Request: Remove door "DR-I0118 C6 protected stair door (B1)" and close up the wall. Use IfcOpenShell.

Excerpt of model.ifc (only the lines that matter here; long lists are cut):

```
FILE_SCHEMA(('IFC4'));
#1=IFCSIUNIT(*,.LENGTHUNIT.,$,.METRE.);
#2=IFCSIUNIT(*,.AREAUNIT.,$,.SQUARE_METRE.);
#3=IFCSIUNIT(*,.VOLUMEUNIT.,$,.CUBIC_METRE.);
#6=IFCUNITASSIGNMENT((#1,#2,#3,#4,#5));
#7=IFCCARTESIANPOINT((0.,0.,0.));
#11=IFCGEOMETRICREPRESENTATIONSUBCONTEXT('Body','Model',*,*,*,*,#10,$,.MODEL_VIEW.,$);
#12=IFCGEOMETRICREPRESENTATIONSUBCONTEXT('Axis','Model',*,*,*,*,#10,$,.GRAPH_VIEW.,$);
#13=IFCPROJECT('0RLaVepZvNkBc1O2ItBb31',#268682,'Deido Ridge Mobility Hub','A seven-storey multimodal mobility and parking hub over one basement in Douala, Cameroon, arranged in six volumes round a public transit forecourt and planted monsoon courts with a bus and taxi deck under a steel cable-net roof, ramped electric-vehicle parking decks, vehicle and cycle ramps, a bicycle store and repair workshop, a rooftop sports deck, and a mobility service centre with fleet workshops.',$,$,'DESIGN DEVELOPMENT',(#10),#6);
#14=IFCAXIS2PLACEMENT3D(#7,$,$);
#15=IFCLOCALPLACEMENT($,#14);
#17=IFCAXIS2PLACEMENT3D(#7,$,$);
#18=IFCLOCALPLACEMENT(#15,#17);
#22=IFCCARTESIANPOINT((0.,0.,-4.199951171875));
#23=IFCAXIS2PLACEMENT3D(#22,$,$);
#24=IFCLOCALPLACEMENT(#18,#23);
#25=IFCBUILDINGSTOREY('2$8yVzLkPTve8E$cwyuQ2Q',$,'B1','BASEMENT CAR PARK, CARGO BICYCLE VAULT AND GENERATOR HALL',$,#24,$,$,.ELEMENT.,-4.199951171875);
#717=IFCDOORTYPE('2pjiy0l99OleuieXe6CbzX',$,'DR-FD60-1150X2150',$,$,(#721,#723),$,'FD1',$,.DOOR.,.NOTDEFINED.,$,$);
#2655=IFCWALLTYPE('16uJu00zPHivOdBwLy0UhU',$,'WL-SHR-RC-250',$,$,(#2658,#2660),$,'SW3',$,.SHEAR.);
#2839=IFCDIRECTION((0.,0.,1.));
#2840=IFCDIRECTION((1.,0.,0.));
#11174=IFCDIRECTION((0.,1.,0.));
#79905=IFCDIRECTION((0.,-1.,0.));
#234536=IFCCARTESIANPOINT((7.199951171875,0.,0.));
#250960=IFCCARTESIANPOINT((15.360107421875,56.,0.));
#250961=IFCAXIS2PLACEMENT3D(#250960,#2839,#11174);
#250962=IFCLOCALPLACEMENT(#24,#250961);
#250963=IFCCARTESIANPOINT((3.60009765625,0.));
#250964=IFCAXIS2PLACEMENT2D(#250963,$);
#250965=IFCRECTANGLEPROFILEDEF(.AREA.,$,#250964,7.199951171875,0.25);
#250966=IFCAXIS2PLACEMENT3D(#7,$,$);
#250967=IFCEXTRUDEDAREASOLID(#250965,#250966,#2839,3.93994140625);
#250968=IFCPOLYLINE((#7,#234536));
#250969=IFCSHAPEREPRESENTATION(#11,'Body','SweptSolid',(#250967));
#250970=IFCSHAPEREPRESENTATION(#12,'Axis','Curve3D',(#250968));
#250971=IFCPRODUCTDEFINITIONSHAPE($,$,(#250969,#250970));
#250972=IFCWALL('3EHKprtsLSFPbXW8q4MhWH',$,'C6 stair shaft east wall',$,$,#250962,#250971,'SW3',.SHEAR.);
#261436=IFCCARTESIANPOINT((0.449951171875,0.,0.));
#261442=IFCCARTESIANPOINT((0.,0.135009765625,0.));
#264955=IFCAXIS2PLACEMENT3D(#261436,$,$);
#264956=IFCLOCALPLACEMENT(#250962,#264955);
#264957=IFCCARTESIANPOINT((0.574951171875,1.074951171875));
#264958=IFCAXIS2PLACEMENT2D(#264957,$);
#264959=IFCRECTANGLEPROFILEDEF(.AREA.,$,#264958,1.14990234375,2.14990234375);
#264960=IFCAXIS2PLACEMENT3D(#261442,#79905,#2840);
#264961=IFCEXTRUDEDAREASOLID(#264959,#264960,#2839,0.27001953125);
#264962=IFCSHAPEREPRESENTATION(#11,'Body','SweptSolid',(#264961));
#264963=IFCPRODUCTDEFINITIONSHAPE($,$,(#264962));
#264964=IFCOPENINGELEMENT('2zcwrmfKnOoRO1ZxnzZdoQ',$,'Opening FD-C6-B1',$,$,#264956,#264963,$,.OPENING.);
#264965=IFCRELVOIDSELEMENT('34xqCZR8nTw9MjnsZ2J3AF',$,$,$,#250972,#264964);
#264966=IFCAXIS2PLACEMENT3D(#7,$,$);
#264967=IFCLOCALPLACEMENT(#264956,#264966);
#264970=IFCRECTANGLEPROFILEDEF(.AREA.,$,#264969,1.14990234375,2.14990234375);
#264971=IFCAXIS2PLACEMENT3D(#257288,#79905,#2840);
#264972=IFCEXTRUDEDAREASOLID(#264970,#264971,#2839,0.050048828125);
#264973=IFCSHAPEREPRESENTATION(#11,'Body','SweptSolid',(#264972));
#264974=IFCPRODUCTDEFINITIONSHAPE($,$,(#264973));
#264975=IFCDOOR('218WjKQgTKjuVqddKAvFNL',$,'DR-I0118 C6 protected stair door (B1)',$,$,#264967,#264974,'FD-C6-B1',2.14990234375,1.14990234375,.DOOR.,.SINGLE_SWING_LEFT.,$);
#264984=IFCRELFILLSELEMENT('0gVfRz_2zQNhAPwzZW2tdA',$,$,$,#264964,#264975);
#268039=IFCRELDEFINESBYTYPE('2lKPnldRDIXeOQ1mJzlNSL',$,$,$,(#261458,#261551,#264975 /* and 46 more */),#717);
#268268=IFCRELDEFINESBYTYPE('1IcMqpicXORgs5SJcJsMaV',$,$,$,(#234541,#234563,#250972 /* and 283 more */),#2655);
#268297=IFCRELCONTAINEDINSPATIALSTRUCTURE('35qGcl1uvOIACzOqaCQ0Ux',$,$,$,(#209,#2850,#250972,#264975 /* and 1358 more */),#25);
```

```python
import ifcopenshell
import ifcopenshell.api.feature
import ifcopenshell.api.root
import ifcopenshell.geom
import ifcopenshell.util.shape

model = ifcopenshell.open("model.ifc")
settings = ifcopenshell.geom.settings()


def volume(element):
    """Net volume in cubic metres, openings subtracted."""
    shape = ifcopenshell.geom.create_shape(settings, element)
    return ifcopenshell.util.shape.get_volume(shape.geometry)


door = model.by_guid("218WjKQgTKjuVqddKAvFNL")
opening = door.FillsVoids[0].RelatingOpeningElement
wall = opening.VoidsElements[0].RelatingBuildingElement
before = volume(wall)

ifcopenshell.api.root.remove_product(model, product=door)
ifcopenshell.api.feature.remove_feature(model, feature=opening)

after = volume(wall)

print(f"wall volume {before:.3f} -> {after:.3f} m3")

model.write("model_updated.ifc")
```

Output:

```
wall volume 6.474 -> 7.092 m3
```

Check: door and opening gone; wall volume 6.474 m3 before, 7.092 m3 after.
